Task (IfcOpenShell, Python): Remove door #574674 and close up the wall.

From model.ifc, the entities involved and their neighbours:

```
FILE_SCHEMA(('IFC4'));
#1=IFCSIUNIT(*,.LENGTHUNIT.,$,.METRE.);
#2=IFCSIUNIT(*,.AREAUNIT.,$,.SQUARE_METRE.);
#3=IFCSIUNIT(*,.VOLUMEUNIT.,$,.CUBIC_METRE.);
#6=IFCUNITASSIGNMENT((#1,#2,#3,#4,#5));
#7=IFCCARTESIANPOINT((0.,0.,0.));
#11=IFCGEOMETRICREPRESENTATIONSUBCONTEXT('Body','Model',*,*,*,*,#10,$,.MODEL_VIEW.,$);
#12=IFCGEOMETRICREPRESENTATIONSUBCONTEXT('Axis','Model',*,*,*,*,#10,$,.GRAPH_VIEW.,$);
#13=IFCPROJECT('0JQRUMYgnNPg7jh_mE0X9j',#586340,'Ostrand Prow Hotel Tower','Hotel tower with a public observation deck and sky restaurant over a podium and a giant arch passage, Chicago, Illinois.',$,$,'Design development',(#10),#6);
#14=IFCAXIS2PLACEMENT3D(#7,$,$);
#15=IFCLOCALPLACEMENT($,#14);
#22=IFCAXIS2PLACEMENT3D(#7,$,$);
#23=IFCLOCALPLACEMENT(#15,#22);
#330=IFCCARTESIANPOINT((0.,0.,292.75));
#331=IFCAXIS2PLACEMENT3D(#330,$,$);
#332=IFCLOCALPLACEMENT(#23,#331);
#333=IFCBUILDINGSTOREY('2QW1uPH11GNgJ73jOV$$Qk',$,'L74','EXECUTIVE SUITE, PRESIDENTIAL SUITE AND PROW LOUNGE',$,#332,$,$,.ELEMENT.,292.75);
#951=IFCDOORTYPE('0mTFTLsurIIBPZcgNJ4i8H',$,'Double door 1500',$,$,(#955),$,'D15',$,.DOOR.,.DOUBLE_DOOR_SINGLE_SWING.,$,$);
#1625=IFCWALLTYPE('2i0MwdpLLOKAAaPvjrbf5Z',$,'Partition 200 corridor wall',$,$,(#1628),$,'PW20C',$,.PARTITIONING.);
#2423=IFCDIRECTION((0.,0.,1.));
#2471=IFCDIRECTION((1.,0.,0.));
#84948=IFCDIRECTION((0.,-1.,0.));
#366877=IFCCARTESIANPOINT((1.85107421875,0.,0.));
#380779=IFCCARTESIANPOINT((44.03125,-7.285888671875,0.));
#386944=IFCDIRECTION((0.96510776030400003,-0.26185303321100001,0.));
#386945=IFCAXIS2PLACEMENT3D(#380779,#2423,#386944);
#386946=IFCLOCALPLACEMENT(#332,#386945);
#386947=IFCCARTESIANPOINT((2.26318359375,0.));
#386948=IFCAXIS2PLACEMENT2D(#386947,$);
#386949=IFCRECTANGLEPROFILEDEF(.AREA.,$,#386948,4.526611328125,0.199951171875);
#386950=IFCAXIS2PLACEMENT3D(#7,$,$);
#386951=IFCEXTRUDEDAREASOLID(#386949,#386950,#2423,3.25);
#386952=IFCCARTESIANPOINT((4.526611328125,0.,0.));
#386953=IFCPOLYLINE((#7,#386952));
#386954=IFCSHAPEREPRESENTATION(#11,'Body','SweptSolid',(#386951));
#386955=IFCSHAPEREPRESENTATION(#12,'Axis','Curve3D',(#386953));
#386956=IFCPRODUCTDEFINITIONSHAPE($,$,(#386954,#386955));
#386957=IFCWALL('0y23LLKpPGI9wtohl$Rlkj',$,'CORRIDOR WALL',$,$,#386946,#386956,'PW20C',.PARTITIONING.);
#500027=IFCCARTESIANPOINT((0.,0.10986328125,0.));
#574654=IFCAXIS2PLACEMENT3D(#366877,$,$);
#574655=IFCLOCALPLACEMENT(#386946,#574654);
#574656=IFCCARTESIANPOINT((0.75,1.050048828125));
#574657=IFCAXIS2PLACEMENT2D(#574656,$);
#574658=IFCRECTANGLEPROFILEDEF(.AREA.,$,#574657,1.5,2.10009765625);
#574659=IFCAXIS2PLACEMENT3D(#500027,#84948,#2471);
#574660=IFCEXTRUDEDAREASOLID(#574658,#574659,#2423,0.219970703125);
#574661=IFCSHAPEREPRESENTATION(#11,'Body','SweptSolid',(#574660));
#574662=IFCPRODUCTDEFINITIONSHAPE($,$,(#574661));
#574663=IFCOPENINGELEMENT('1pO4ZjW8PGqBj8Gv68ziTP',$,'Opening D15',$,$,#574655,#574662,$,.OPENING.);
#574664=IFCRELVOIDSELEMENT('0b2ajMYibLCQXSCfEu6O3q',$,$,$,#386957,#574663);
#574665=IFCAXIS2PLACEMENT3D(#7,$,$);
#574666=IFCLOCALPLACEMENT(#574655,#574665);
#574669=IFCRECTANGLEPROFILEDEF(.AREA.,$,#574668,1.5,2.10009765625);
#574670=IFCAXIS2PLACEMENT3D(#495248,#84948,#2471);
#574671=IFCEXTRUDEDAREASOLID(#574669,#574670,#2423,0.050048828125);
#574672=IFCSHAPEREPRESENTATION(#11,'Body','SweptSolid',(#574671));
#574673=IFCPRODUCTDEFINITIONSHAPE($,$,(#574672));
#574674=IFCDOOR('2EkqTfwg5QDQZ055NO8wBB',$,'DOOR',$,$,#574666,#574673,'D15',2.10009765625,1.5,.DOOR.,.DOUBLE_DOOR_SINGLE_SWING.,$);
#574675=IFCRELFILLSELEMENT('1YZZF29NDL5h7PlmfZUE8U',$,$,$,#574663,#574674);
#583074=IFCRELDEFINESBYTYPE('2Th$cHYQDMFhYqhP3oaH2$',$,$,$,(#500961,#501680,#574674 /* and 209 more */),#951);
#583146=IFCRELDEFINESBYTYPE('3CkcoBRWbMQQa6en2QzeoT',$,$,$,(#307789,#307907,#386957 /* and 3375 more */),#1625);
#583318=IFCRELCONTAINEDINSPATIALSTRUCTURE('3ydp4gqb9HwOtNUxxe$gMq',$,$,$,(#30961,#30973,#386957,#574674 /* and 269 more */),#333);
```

```python
import ifcopenshell
import ifcopenshell.api.feature
import ifcopenshell.api.root
import ifcopenshell.geom
import ifcopenshell.util.shape

model = ifcopenshell.open("model.ifc")
settings = ifcopenshell.geom.settings()


def volume(element):
    """Net volume in cubic metres, openings subtracted."""
    shape = ifcopenshell.geom.create_shape(settings, element)
    return ifcopenshell.util.shape.get_volume(shape.geometry)


door = model.by_guid("2EkqTfwg5QDQZ055NO8wBB")
opening = door.FillsVoids[0].RelatingOpeningElement
wall = opening.VoidsElements[0].RelatingBuildingElement
before = volume(wall)

ifcopenshell.api.root.remove_product(model, product=door)
ifcopenshell.api.feature.remove_feature(model, feature=opening)

after = volume(wall)

print(f"wall volume {before:.3f} -> {after:.3f} m3")

model.write("model_v2.ifc")
```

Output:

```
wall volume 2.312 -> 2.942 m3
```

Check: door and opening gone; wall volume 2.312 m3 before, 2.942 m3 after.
